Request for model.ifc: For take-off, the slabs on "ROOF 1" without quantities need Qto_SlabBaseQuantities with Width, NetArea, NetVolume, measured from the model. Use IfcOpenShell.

First a look at what the model holds.

```python
import ifcopenshell
import ifcopenshell.util.element
import ifcopenshell.util.unit

model = ifcopenshell.open("model.ifc")
print(model.schema)
for unit_type in ("LENGTHUNIT", "AREAUNIT", "VOLUMEUNIT"):
    print(unit_type, ifcopenshell.util.unit.calculate_unit_scale(model, unit_type))
storey = next(s for s in model.by_type("IfcBuildingStorey") if s.Name == "ROOF 1")
slabs = [e for e in ifcopenshell.util.element.get_decomposition(storey) if e.is_a("IfcSlab")]
for e in sorted(slabs, key=lambda e: e.id()):
    print(e.id(), e.is_a(), e.Name, list(ifcopenshell.util.element.get_psets(e, qtos_only=True)), sep=" | ")
```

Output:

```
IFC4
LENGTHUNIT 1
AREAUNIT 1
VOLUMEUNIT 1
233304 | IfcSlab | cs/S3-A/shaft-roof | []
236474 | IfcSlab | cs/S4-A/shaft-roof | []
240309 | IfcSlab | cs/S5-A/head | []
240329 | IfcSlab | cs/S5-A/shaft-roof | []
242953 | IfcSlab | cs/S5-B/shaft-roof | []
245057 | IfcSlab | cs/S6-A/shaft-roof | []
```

```python
import ifcopenshell
import ifcopenshell.api.pset
import ifcopenshell.geom
import ifcopenshell.util.element
import ifcopenshell.util.shape
import ifcopenshell.util.unit

model = ifcopenshell.open("model.ifc")
unit_scale = ifcopenshell.util.unit.calculate_unit_scale(model)
area_scale = ifcopenshell.util.unit.calculate_unit_scale(model, "AREAUNIT")
volume_scale = ifcopenshell.util.unit.calculate_unit_scale(model, "VOLUMEUNIT")
settings = ifcopenshell.geom.settings()

storey = next(s for s in model.by_type("IfcBuildingStorey") if s.Name == "ROOF 1")
slabs = [e for e in ifcopenshell.util.element.get_decomposition(storey) if e.is_a("IfcSlab")]

for e in sorted(slabs, key=lambda e: e.id()):
    if ifcopenshell.util.element.get_psets(e, qtos_only=True, should_inherit=False):
        continue
    # Geometry comes back in metres, in the element's own axes.
    shape = ifcopenshell.geom.create_shape(settings, e)
    values = {
        "Width": ifcopenshell.util.shape.get_z(shape.geometry) / unit_scale,
        "NetArea": ifcopenshell.util.shape.get_footprint_area(shape.geometry) / area_scale,
        "NetVolume": ifcopenshell.util.shape.get_volume(shape.geometry) / volume_scale,
    }
    qto = ifcopenshell.api.pset.add_qto(model, product=e, name="Qto_SlabBaseQuantities")
    ifcopenshell.api.pset.edit_qto(model, qto=qto, properties=values)
    print(e.id(), {k: round(v, 3) for k, v in values.items()})

model.write("model_edited.ifc")
```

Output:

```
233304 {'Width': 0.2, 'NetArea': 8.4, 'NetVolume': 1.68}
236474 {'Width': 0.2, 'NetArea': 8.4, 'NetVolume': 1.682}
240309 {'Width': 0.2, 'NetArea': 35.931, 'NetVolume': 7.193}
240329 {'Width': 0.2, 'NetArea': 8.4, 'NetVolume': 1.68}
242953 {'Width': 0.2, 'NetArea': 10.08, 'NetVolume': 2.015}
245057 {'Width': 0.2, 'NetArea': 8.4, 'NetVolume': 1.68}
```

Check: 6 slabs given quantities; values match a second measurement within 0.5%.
